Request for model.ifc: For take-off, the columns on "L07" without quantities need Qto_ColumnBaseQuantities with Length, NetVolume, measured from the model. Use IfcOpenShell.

First a look at what the model holds.

```python
import ifcopenshell
import ifcopenshell.util.element
import ifcopenshell.util.unit

model = ifcopenshell.open("model.ifc")
print(model.schema)
for unit_type in ("LENGTHUNIT", "AREAUNIT", "VOLUMEUNIT"):
    print(unit_type, ifcopenshell.util.unit.calculate_unit_scale(model, unit_type))
storey = next(s for s in model.by_type("IfcBuildingStorey") if s.Name == "L07")
columns = [e for e in ifcopenshell.util.element.get_decomposition(storey) if e.is_a("IfcColumn")]
for e in sorted(columns, key=lambda e: e.id()):
    print(e.id(), e.is_a(), e.Name, list(ifcopenshell.util.element.get_psets(e, qtos_only=True)), sep=" | ")
```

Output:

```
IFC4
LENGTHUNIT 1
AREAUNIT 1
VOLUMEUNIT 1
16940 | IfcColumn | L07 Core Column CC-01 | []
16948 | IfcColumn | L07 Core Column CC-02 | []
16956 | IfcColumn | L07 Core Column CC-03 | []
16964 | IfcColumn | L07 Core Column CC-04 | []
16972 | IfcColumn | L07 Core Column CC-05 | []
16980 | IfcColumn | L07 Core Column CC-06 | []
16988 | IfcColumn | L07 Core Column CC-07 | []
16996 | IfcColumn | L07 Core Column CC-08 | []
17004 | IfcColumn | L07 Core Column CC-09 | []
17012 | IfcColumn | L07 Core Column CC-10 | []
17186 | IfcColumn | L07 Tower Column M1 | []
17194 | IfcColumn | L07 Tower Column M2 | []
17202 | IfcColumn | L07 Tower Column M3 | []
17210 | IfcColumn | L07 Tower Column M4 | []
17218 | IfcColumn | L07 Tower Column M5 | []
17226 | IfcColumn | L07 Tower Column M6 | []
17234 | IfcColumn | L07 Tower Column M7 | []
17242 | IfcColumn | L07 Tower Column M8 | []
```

```python
import ifcopenshell
import ifcopenshell.api.pset
import ifcopenshell.geom
import ifcopenshell.util.element
import ifcopenshell.util.shape
import ifcopenshell.util.unit

model = ifcopenshell.open("model.ifc")
unit_scale = ifcopenshell.util.unit.calculate_unit_scale(model)
volume_scale = ifcopenshell.util.unit.calculate_unit_scale(model, "VOLUMEUNIT")
settings = ifcopenshell.geom.settings()

storey = next(s for s in model.by_type("IfcBuildingStorey") if s.Name == "L07")
columns = [e for e in ifcopenshell.util.element.get_decomposition(storey) if e.is_a("IfcColumn")]

for e in sorted(columns, key=lambda e: e.id()):
    if ifcopenshell.util.element.get_psets(e, qtos_only=True, should_inherit=False):
        continue
    # Geometry comes back in metres, in the element's own axes.
    shape = ifcopenshell.geom.create_shape(settings, e)
    values = {
        "Length": ifcopenshell.util.shape.get_z(shape.geometry) / unit_scale,
        "NetVolume": ifcopenshell.util.shape.get_volume(shape.geometry) / volume_scale,
    }
    qto = ifcopenshell.api.pset.add_qto(model, product=e, name="Qto_ColumnBaseQuantities")
    ifcopenshell.api.pset.edit_qto(model, qto=qto, properties=values)
    print(e.id(), {k: round(v, 3) for k, v in values.items()})

model.write("model_rev.ifc")
```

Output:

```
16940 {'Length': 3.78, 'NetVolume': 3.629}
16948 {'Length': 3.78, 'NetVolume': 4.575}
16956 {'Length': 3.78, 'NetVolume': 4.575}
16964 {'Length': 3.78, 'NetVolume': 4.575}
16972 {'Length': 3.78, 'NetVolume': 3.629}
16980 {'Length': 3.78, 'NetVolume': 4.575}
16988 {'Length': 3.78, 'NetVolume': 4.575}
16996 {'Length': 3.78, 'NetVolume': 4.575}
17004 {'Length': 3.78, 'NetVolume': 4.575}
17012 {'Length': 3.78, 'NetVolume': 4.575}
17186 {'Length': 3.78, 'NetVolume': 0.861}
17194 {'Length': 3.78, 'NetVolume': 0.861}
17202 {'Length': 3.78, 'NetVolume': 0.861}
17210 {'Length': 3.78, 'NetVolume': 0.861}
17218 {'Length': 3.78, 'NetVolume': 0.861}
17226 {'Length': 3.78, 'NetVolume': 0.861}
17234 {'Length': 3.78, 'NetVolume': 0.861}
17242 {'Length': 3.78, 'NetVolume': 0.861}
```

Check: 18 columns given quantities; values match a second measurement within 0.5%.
